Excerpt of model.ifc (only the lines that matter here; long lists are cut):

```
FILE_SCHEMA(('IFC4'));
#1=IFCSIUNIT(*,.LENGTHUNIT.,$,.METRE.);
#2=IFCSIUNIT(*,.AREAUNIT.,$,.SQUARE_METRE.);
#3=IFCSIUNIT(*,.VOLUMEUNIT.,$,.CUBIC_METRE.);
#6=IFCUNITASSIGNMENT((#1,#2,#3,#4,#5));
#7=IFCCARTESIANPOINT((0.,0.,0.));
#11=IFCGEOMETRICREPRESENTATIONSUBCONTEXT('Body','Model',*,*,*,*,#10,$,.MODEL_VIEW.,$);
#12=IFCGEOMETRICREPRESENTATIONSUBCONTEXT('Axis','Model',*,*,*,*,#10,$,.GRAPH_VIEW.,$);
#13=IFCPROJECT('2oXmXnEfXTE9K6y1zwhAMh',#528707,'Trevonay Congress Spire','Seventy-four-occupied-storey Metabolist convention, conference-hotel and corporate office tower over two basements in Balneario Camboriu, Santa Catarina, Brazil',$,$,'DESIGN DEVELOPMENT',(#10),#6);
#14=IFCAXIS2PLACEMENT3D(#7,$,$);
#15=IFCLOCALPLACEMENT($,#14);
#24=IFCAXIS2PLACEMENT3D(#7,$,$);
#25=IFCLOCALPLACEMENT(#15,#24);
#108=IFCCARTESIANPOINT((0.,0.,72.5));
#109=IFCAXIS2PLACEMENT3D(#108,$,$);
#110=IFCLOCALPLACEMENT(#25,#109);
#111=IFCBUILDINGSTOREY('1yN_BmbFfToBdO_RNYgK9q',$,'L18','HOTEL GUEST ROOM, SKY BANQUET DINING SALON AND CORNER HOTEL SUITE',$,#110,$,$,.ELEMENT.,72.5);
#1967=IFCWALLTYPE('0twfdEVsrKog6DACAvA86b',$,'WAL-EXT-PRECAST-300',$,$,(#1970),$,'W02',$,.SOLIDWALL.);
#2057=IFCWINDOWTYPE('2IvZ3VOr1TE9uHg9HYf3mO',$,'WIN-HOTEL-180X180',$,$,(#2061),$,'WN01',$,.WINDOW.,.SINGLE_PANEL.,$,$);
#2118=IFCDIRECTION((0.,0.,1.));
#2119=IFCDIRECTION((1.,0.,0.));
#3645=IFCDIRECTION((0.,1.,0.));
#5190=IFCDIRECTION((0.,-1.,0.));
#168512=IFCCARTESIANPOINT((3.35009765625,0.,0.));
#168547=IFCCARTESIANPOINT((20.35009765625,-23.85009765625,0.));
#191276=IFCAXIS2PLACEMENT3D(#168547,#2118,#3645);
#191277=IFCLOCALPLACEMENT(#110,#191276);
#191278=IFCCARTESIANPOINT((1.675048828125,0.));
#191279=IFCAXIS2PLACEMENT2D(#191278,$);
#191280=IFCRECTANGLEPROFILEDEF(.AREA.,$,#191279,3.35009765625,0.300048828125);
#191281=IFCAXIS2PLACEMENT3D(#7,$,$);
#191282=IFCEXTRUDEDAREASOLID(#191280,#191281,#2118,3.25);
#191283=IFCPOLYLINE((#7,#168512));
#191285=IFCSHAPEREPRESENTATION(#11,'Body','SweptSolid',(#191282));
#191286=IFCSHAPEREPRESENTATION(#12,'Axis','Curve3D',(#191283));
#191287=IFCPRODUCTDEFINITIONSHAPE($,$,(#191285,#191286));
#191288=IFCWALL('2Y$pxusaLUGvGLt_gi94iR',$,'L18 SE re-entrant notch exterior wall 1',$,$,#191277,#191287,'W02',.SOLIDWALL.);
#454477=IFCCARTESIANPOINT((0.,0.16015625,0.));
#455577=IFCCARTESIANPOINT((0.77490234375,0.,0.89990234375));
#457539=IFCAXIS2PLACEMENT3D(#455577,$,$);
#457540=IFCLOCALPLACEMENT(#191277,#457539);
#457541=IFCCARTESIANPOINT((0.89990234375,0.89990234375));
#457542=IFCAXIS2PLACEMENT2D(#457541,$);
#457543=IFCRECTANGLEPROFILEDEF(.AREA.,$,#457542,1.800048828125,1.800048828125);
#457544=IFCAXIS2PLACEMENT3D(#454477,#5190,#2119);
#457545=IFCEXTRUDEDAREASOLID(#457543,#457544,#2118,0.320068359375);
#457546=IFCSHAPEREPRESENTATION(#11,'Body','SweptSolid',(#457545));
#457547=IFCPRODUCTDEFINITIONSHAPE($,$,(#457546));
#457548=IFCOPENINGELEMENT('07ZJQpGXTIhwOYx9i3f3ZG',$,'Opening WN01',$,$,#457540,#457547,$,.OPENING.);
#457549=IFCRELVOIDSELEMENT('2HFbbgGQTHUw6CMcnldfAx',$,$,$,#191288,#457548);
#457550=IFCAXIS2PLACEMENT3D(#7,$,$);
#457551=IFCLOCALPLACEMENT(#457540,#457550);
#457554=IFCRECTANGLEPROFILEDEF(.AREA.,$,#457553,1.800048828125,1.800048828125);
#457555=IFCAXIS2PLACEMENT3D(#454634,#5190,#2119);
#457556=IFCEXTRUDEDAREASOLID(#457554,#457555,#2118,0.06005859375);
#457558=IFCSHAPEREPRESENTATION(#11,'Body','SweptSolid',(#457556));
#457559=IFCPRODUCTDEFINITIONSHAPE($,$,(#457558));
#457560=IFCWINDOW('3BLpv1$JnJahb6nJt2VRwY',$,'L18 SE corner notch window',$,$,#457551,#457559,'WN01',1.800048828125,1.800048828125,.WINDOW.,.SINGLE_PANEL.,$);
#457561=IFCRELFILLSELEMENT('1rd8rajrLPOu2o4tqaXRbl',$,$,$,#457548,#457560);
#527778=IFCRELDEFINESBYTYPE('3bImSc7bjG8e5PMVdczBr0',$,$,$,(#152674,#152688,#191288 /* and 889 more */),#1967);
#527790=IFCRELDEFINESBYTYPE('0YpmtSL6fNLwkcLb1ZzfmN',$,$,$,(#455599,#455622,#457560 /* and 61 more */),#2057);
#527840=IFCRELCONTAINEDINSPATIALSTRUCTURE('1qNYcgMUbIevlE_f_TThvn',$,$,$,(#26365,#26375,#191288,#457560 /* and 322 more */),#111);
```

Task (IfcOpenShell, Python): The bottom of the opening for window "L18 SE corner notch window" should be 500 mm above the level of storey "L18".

```python
import numpy as np
import ifcopenshell
import ifcopenshell.api.geometry
import ifcopenshell.geom
import ifcopenshell.util.element
import ifcopenshell.util.placement
import ifcopenshell.util.shape
import ifcopenshell.util.unit

model = ifcopenshell.open("model.ifc")
unit_scale = ifcopenshell.util.unit.calculate_unit_scale(model)

window = model.by_guid("3BLpv1$JnJahb6nJt2VRwY")
opening = window.FillsVoids[0].RelatingOpeningElement
storey = ifcopenshell.util.element.get_container(window, ifc_class="IfcBuildingStorey")
level = ifcopenshell.util.placement.get_local_placement(storey.ObjectPlacement)[2, 3]

# The opening's origin need not be at the sill, so measure its lowest point.
shape = ifcopenshell.geom.create_shape(ifcopenshell.geom.settings(), opening)
bottom = ifcopenshell.util.shape.get_shape_bottom_elevation(shape, shape.geometry) / unit_scale
dz = level + 0.5 / unit_scale - bottom

shift = np.array([0.0, 0.0, dz])
# The window is placed relative to its opening, so it follows when the opening moves.
matrix = ifcopenshell.util.placement.get_local_placement(opening.ObjectPlacement)
matrix[:3, 3] += shift
ifcopenshell.api.geometry.edit_object_placement(
    model, product=opening, matrix=matrix, is_si=False, should_transform_children=True
)

print(f"moved by {dz * unit_scale:+.3f} m")

model.write("model_v2.ifc")
```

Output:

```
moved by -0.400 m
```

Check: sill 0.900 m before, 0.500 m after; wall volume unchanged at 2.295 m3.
